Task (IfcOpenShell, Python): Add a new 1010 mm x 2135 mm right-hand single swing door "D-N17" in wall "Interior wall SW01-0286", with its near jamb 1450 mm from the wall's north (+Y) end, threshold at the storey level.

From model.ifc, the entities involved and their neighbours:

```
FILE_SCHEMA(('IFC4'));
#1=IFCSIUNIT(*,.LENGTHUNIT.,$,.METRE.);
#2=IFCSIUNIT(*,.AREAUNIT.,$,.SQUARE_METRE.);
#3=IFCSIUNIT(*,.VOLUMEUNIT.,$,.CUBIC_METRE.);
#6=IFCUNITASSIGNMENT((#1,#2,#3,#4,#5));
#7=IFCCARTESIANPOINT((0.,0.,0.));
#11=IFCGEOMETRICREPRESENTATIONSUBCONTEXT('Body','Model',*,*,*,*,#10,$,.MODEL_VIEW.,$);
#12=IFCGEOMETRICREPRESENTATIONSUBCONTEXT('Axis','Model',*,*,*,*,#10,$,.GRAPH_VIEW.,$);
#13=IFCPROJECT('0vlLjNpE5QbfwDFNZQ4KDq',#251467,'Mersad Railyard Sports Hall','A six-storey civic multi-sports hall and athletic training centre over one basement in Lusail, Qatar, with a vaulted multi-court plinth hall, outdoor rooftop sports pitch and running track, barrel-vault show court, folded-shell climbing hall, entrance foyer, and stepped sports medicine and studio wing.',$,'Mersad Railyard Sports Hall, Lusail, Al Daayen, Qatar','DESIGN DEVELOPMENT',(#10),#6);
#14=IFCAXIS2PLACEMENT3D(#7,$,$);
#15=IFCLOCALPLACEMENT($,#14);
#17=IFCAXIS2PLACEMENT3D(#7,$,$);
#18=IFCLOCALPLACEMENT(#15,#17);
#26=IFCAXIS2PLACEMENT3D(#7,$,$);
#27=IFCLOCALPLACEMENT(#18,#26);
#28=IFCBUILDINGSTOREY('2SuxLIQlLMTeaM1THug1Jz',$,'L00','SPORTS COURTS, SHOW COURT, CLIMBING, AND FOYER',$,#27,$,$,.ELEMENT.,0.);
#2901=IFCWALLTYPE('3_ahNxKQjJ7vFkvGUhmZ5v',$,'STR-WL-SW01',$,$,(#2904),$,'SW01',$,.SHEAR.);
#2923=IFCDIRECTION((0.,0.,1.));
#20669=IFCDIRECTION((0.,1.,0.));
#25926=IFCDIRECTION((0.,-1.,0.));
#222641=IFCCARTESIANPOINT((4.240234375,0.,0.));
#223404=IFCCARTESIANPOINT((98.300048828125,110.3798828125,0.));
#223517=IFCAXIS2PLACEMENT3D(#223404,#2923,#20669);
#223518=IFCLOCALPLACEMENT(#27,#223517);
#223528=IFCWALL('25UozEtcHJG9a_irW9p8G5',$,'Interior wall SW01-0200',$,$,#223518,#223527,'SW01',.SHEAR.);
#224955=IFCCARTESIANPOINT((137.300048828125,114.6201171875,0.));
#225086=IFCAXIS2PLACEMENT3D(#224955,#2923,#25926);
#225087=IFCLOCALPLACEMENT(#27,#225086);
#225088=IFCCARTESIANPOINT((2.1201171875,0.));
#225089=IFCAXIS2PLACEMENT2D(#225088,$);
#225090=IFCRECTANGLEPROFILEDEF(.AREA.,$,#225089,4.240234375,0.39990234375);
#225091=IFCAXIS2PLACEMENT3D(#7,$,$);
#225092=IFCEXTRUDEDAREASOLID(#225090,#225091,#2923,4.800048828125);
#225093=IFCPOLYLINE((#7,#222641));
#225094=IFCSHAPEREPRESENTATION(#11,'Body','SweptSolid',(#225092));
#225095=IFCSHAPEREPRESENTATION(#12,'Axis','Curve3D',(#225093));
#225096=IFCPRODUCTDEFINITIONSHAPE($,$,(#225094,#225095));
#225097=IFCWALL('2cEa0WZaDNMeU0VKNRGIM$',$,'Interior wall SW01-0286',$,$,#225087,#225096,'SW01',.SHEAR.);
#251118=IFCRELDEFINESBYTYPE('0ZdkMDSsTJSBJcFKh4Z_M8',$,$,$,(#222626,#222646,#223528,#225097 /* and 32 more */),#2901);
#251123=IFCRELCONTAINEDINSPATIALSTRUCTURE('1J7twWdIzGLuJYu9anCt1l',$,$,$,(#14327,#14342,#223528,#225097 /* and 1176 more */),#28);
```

```python
import numpy as np
import ifcopenshell
import ifcopenshell.api.feature
import ifcopenshell.api.geometry
import ifcopenshell.api.root
import ifcopenshell.api.spatial
import ifcopenshell.geom
import ifcopenshell.util.element
import ifcopenshell.util.placement
import ifcopenshell.util.representation
import ifcopenshell.util.shape
import ifcopenshell.util.unit

model = ifcopenshell.open("model.ifc")
unit_scale = ifcopenshell.util.unit.calculate_unit_scale(model)
settings = ifcopenshell.geom.settings()


def volume(element):
    """Net volume in cubic metres, openings subtracted."""
    shape = ifcopenshell.geom.create_shape(settings, element)
    return ifcopenshell.util.shape.get_volume(shape.geometry)


wall = model.by_id(225097)
storey = ifcopenshell.util.element.get_container(wall, ifc_class="IfcBuildingStorey")
context = ifcopenshell.util.representation.get_context(model, "Model", "Body", "MODEL_VIEW")
before = volume(wall)

width, height, from_end, sill = 1.01, 2.135, 1.45, 0.0  # metres

# The wall runs along its own X axis, and the end named is its -X end.
wall_shape = ifcopenshell.geom.create_shape(settings, wall)
x, y, z = ifcopenshell.util.shape.get_vertices(wall_shape.geometry).T
start = x.min() + from_end
face, thickness = float(y.min()), float(y.max() - y.min())
wall_matrix = ifcopenshell.util.placement.get_local_placement(wall.ObjectPlacement)
level = ifcopenshell.util.placement.get_local_placement(storey.ObjectPlacement)[2, 3]


def in_wall(x, y):
    """Placement at x, y metres in the wall's axes, at sill height."""
    matrix = wall_matrix.copy()
    matrix[:, 3] = wall_matrix @ np.array([x / unit_scale, y / unit_scale, 0.0, 1.0])
    matrix[2, 3] = level + sill / unit_scale
    return matrix


# Opening: a box that overshoots both wall faces by 50 mm.
opening = ifcopenshell.api.root.create_entity(model, ifc_class="IfcOpeningElement", predefined_type="OPENING")
box = ifcopenshell.api.geometry.add_wall_representation(
    model, context=context, length=width, height=height, thickness=thickness + 0.1
)
ifcopenshell.api.geometry.assign_representation(model, product=opening, representation=box)
ifcopenshell.api.geometry.edit_object_placement(model, product=opening, matrix=in_wall(start, face - 0.05), is_si=False)
ifcopenshell.api.feature.add_feature(model, feature=opening, element=wall)

door = ifcopenshell.api.root.create_entity(model, ifc_class="IfcDoor", name="D-N17", predefined_type="DOOR")
door.OverallWidth, door.OverallHeight = width / unit_scale, height / unit_scale
door.OperationType = "SINGLE_SWING_RIGHT"
body = ifcopenshell.api.geometry.add_door_representation(
    model,
    context=context,
    overall_width=door.OverallWidth,
    overall_height=door.OverallHeight,
    operation_type="SINGLE_SWING_RIGHT",
    lining_properties={"LiningDepth": thickness / unit_scale, "ThresholdDepth": thickness / unit_scale},
)
ifcopenshell.api.geometry.assign_representation(model, product=door, representation=body)
ifcopenshell.api.spatial.assign_container(model, products=[door], relating_structure=storey)
ifcopenshell.api.feature.add_filling(model, opening=opening, element=door)

# The lining spans the wall, so the door starts at the wall face.
ifcopenshell.api.geometry.edit_object_placement(model, product=door, matrix=in_wall(start, face), is_si=False)

after = volume(wall)

print(f"wall volume {before:.3f} -> {after:.3f} m3")

model.write("model-out.ifc")
```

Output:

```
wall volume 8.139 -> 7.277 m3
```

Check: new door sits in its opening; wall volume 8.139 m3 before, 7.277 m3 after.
